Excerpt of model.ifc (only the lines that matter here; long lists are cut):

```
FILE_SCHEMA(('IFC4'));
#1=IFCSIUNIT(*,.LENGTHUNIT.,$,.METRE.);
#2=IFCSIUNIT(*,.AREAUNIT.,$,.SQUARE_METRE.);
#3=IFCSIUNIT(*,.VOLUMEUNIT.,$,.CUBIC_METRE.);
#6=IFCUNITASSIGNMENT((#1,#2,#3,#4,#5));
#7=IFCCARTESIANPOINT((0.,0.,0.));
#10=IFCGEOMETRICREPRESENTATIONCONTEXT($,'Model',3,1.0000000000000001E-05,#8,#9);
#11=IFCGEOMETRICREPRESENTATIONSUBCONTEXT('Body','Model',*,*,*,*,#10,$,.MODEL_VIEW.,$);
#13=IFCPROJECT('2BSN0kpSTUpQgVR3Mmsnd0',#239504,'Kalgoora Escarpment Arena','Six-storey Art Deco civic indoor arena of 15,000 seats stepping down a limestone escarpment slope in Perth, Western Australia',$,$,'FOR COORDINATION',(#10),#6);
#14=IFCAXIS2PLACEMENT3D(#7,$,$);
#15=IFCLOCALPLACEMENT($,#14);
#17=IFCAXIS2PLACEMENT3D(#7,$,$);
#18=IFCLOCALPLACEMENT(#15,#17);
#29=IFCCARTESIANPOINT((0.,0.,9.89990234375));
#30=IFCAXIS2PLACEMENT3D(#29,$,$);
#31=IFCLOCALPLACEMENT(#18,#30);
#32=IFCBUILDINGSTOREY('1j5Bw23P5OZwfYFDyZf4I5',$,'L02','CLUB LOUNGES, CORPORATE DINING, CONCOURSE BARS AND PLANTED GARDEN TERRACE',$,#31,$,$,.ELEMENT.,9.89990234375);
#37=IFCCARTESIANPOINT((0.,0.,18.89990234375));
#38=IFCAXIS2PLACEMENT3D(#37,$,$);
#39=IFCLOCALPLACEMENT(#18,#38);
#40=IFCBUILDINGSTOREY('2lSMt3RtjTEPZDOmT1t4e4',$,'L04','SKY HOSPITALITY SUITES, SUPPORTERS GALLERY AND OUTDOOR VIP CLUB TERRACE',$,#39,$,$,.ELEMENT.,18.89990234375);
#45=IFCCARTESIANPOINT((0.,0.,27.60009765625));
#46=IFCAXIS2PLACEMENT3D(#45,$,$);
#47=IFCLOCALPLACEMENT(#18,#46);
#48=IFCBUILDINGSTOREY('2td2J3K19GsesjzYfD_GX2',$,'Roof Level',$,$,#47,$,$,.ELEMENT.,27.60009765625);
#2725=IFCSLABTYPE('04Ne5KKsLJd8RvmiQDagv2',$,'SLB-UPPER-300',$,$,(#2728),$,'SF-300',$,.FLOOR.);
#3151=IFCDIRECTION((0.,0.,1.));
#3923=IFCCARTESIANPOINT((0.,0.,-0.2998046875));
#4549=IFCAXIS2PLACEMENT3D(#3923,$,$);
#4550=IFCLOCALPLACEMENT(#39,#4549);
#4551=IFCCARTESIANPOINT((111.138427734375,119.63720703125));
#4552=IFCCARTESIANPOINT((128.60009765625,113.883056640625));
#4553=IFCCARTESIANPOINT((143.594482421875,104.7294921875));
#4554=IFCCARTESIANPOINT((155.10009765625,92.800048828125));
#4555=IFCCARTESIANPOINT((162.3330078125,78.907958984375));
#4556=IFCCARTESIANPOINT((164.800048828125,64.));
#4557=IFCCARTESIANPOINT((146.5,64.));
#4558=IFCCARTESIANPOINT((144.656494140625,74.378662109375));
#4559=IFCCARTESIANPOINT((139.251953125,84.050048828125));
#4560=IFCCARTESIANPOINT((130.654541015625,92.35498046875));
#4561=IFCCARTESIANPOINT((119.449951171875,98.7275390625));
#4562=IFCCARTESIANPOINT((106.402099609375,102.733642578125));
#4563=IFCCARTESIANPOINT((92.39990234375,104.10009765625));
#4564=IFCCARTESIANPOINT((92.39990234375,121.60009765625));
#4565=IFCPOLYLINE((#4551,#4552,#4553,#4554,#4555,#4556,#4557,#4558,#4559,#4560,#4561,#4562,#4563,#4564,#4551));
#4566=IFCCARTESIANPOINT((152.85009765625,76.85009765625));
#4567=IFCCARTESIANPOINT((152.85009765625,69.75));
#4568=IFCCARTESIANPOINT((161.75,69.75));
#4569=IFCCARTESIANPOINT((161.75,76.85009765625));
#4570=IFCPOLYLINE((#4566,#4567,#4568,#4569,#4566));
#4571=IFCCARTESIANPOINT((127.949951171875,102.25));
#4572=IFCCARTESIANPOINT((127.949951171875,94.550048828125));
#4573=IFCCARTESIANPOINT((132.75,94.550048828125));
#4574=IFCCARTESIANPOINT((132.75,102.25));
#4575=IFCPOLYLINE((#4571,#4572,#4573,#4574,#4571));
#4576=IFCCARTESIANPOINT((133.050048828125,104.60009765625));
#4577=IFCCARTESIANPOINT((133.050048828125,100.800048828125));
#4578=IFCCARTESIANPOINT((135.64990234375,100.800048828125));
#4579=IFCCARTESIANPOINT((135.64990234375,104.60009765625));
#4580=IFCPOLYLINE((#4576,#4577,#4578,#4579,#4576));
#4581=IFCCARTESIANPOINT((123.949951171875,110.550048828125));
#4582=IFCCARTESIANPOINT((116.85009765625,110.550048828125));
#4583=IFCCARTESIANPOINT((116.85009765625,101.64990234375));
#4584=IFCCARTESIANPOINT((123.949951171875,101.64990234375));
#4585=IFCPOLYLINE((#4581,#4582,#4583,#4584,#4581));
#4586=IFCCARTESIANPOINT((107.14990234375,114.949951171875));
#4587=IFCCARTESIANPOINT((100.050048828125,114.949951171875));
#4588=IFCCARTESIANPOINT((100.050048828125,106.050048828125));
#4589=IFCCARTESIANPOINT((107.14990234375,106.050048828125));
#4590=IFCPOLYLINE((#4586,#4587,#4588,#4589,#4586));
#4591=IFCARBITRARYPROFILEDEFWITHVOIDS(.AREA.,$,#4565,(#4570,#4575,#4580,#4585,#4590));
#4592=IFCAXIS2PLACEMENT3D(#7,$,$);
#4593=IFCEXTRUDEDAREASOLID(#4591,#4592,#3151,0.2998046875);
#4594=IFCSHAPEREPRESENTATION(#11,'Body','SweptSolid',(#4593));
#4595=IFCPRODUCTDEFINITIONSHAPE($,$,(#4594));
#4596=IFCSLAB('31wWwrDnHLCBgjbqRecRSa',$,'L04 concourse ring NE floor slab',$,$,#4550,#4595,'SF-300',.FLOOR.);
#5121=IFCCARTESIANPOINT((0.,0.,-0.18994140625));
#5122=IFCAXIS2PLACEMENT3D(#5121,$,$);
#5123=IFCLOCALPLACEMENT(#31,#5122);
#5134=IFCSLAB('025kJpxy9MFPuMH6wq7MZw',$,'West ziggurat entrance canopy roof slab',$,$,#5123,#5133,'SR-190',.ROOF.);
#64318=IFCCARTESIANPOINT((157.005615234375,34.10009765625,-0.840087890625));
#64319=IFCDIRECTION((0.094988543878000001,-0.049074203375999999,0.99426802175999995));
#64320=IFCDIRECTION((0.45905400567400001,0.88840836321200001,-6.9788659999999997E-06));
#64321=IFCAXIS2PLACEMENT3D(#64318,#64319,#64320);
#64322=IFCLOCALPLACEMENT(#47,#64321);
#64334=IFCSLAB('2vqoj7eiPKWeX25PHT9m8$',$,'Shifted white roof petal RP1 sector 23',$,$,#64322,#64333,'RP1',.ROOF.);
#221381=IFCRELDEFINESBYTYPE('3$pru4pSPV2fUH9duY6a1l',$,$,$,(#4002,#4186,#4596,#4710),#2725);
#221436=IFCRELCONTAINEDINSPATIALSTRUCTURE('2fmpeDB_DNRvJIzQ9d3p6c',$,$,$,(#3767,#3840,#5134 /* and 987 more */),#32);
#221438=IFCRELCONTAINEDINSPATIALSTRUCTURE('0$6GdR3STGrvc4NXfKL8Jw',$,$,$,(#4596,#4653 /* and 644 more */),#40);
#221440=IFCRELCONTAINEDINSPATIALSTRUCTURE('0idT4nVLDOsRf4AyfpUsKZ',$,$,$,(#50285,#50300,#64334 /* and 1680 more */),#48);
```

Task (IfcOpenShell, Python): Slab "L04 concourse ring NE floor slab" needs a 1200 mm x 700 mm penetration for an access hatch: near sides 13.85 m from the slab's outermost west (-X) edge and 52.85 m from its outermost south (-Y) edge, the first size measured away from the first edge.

```python
import numpy as np
import ifcopenshell
import ifcopenshell.api.feature
import ifcopenshell.api.geometry
import ifcopenshell.api.root
import ifcopenshell.geom
import ifcopenshell.util.placement
import ifcopenshell.util.representation
import ifcopenshell.util.shape
import ifcopenshell.util.unit

model = ifcopenshell.open("model.ifc")
unit_scale = ifcopenshell.util.unit.calculate_unit_scale(model)
settings = ifcopenshell.geom.settings()


def volume(element):
    """Net volume in cubic metres, openings subtracted."""
    shape = ifcopenshell.geom.create_shape(settings, element)
    return ifcopenshell.util.shape.get_volume(shape.geometry)


slab = model.by_guid("31wWwrDnHLCBgjbqRecRSa")
before = volume(slab)

# Extent in the slab's own axes, in metres. The edges named are its -X and -Y sides.
slab_shape = ifcopenshell.geom.create_shape(settings, slab)
vertices = ifcopenshell.util.shape.get_vertices(slab_shape.geometry)
x_min, y_min, bottom = vertices.min(axis=0)
top = vertices[:, 2].max()

opening = ifcopenshell.api.root.create_entity(model, ifc_class="IfcOpeningElement", name="Access hatch opening", predefined_type="OPENING")
context = ifcopenshell.util.representation.get_context(model, "Model", "Body", "MODEL_VIEW")
width, depth = 1.2, 0.7
outline = [(0.0, 0.0), (width, 0.0), (width, depth), (0.0, depth), (0.0, 0.0)]
# Overshoot both faces by 50 mm so the cut is clean.
shape = ifcopenshell.api.geometry.add_slab_representation(
    model, context=context, depth=top - bottom + 0.1, polyline=outline
)
ifcopenshell.api.geometry.assign_representation(model, product=opening, representation=shape)

matrix = ifcopenshell.util.placement.get_local_placement(slab.ObjectPlacement)
matrix[:, 3] = matrix @ np.append(np.array([x_min + 13.85, y_min + 52.85, bottom - 0.05]) / unit_scale, 1.0)
ifcopenshell.api.geometry.edit_object_placement(model, product=opening, matrix=matrix, is_si=False)
ifcopenshell.api.feature.add_feature(model, feature=opening, element=slab)

after = volume(slab)

print(f"slab volume {before:.3f} -> {after:.3f} m3")

model.write("model_updated.ifc")
```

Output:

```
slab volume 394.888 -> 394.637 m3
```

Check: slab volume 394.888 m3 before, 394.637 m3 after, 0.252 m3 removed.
